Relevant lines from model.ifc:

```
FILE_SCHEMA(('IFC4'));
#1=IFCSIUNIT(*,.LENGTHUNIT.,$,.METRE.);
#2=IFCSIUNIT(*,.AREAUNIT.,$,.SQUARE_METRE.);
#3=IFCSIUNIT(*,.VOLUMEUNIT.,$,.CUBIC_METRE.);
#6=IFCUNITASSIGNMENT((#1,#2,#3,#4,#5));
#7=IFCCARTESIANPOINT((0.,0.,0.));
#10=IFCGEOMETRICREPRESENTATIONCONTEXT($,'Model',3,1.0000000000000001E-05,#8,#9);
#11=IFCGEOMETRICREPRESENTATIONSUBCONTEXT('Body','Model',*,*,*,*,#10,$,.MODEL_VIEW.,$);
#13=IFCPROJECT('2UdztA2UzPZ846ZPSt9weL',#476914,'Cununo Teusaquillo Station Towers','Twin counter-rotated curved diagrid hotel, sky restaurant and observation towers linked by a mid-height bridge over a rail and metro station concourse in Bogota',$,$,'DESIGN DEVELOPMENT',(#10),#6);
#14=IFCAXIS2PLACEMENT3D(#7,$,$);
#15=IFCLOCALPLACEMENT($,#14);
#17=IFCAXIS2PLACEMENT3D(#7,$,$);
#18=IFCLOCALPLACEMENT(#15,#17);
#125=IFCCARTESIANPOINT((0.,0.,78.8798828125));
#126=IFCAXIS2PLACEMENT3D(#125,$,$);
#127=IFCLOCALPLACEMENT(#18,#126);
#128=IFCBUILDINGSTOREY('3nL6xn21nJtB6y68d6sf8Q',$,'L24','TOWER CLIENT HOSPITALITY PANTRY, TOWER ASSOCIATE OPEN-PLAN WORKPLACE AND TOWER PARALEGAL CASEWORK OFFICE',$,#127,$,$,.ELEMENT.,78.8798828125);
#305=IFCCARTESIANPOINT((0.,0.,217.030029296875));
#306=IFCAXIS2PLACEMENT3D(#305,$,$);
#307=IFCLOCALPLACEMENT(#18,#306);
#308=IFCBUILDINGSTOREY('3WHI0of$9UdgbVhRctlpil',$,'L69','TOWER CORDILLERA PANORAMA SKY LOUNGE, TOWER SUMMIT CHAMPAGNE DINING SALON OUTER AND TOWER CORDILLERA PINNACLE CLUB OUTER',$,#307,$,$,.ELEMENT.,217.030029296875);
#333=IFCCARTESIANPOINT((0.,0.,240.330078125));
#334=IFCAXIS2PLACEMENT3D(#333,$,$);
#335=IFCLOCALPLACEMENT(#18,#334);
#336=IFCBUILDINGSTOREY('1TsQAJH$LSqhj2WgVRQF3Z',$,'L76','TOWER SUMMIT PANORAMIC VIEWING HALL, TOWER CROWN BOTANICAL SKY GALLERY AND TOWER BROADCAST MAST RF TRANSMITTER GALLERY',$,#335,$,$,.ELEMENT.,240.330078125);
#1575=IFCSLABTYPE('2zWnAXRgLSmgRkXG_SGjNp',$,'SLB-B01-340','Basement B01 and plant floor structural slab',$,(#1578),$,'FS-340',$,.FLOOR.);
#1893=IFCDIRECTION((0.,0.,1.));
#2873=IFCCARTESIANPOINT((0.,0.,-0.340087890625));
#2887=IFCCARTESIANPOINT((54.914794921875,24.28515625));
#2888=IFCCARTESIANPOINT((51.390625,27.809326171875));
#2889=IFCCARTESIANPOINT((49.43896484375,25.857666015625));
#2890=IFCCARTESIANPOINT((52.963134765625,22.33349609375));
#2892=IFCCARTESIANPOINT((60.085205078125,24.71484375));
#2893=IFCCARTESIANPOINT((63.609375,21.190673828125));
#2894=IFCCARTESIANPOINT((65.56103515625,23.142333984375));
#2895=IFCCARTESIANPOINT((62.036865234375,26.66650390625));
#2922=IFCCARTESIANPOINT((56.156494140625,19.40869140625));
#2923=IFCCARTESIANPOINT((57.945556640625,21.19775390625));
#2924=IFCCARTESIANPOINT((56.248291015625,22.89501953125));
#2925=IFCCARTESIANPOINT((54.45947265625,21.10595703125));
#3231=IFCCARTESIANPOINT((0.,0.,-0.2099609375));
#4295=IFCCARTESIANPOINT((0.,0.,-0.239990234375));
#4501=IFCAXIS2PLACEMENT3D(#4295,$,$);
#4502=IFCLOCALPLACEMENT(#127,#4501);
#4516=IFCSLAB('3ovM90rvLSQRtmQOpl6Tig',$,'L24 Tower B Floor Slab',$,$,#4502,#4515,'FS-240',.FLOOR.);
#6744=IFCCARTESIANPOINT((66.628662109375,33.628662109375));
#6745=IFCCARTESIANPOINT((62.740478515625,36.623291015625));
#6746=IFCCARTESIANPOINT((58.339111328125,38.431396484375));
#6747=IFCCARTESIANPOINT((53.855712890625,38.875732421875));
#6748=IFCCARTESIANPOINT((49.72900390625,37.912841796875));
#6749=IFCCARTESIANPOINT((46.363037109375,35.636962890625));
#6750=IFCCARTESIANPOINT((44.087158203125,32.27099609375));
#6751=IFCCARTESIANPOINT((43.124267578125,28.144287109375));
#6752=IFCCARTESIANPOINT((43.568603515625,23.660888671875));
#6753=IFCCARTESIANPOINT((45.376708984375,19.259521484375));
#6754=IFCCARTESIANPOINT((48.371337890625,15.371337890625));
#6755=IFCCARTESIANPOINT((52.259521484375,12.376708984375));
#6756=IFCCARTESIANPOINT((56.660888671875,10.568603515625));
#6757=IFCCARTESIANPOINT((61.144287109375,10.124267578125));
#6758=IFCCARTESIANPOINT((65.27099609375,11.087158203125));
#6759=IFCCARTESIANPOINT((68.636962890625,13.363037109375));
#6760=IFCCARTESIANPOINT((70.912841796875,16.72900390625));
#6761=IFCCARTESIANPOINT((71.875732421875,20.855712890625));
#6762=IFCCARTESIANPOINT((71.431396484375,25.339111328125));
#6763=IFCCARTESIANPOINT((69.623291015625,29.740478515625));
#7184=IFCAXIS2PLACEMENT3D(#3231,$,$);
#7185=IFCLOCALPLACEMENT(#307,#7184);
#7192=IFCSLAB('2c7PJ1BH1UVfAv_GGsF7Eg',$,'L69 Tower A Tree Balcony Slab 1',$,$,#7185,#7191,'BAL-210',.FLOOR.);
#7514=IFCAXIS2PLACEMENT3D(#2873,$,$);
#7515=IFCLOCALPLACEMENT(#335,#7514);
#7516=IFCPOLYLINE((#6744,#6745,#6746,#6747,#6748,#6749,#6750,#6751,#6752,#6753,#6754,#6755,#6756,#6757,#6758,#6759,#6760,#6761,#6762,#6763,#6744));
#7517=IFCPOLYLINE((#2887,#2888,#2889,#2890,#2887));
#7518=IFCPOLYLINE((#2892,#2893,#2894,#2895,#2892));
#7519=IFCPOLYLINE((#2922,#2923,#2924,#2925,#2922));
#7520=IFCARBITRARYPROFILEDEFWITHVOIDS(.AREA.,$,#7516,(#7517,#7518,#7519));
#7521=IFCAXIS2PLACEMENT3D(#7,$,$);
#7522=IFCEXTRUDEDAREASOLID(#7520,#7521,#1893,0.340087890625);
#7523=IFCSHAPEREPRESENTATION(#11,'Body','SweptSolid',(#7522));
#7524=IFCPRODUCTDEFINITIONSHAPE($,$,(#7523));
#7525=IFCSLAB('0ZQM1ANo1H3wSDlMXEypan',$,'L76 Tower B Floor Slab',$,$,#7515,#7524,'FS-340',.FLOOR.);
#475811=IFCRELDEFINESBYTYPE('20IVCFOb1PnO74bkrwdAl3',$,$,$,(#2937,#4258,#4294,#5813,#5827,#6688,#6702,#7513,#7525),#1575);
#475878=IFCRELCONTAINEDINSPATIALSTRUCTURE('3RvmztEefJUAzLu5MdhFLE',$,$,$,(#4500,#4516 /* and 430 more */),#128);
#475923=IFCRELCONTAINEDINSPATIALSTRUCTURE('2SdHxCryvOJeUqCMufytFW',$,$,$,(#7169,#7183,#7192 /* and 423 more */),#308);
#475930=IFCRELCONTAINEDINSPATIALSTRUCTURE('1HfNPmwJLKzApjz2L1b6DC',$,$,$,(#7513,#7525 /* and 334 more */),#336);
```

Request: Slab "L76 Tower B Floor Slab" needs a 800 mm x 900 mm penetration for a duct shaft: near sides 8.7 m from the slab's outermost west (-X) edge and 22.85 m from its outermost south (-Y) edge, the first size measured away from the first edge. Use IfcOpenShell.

```python
import numpy as np
import ifcopenshell
import ifcopenshell.api.feature
import ifcopenshell.api.geometry
import ifcopenshell.api.root
import ifcopenshell.geom
import ifcopenshell.util.placement
import ifcopenshell.util.representation
import ifcopenshell.util.shape
import ifcopenshell.util.unit

model = ifcopenshell.open("model.ifc")
unit_scale = ifcopenshell.util.unit.calculate_unit_scale(model)
settings = ifcopenshell.geom.settings()


def volume(element):
    """Net volume in cubic metres, openings subtracted."""
    shape = ifcopenshell.geom.create_shape(settings, element)
    return ifcopenshell.util.shape.get_volume(shape.geometry)


slab = model.by_guid("0ZQM1ANo1H3wSDlMXEypan")
before = volume(slab)

# Extent in the slab's own axes, in metres. The edges named are its -X and -Y sides.
slab_shape = ifcopenshell.geom.create_shape(settings, slab)
vertices = ifcopenshell.util.shape.get_vertices(slab_shape.geometry)
x_min, y_min, bottom = vertices.min(axis=0)
top = vertices[:, 2].max()

opening = ifcopenshell.api.root.create_entity(model, ifc_class="IfcOpeningElement", name="Duct shaft opening", predefined_type="OPENING")
context = ifcopenshell.util.representation.get_context(model, "Model", "Body", "MODEL_VIEW")
width, depth = 0.8, 0.9
outline = [(0.0, 0.0), (width, 0.0), (width, depth), (0.0, depth), (0.0, 0.0)]
# Overshoot both faces by 50 mm so the cut is clean.
shape = ifcopenshell.api.geometry.add_slab_representation(
    model, context=context, depth=top - bottom + 0.1, polyline=outline
)
ifcopenshell.api.geometry.assign_representation(model, product=opening, representation=shape)

matrix = ifcopenshell.util.placement.get_local_placement(slab.ObjectPlacement)
matrix[:, 3] = matrix @ np.append(np.array([x_min + 8.7, y_min + 22.85, bottom - 0.05]) / unit_scale, 1.0)
ifcopenshell.api.geometry.edit_object_placement(model, product=opening, matrix=matrix, is_si=False)
ifcopenshell.api.feature.add_feature(model, feature=opening, element=slab)

after = volume(slab)

print(f"slab volume {before:.3f} -> {after:.3f} m3")

model.write("model_rev.ifc")
```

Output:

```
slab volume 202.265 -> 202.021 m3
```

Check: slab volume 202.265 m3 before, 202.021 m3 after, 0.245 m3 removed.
